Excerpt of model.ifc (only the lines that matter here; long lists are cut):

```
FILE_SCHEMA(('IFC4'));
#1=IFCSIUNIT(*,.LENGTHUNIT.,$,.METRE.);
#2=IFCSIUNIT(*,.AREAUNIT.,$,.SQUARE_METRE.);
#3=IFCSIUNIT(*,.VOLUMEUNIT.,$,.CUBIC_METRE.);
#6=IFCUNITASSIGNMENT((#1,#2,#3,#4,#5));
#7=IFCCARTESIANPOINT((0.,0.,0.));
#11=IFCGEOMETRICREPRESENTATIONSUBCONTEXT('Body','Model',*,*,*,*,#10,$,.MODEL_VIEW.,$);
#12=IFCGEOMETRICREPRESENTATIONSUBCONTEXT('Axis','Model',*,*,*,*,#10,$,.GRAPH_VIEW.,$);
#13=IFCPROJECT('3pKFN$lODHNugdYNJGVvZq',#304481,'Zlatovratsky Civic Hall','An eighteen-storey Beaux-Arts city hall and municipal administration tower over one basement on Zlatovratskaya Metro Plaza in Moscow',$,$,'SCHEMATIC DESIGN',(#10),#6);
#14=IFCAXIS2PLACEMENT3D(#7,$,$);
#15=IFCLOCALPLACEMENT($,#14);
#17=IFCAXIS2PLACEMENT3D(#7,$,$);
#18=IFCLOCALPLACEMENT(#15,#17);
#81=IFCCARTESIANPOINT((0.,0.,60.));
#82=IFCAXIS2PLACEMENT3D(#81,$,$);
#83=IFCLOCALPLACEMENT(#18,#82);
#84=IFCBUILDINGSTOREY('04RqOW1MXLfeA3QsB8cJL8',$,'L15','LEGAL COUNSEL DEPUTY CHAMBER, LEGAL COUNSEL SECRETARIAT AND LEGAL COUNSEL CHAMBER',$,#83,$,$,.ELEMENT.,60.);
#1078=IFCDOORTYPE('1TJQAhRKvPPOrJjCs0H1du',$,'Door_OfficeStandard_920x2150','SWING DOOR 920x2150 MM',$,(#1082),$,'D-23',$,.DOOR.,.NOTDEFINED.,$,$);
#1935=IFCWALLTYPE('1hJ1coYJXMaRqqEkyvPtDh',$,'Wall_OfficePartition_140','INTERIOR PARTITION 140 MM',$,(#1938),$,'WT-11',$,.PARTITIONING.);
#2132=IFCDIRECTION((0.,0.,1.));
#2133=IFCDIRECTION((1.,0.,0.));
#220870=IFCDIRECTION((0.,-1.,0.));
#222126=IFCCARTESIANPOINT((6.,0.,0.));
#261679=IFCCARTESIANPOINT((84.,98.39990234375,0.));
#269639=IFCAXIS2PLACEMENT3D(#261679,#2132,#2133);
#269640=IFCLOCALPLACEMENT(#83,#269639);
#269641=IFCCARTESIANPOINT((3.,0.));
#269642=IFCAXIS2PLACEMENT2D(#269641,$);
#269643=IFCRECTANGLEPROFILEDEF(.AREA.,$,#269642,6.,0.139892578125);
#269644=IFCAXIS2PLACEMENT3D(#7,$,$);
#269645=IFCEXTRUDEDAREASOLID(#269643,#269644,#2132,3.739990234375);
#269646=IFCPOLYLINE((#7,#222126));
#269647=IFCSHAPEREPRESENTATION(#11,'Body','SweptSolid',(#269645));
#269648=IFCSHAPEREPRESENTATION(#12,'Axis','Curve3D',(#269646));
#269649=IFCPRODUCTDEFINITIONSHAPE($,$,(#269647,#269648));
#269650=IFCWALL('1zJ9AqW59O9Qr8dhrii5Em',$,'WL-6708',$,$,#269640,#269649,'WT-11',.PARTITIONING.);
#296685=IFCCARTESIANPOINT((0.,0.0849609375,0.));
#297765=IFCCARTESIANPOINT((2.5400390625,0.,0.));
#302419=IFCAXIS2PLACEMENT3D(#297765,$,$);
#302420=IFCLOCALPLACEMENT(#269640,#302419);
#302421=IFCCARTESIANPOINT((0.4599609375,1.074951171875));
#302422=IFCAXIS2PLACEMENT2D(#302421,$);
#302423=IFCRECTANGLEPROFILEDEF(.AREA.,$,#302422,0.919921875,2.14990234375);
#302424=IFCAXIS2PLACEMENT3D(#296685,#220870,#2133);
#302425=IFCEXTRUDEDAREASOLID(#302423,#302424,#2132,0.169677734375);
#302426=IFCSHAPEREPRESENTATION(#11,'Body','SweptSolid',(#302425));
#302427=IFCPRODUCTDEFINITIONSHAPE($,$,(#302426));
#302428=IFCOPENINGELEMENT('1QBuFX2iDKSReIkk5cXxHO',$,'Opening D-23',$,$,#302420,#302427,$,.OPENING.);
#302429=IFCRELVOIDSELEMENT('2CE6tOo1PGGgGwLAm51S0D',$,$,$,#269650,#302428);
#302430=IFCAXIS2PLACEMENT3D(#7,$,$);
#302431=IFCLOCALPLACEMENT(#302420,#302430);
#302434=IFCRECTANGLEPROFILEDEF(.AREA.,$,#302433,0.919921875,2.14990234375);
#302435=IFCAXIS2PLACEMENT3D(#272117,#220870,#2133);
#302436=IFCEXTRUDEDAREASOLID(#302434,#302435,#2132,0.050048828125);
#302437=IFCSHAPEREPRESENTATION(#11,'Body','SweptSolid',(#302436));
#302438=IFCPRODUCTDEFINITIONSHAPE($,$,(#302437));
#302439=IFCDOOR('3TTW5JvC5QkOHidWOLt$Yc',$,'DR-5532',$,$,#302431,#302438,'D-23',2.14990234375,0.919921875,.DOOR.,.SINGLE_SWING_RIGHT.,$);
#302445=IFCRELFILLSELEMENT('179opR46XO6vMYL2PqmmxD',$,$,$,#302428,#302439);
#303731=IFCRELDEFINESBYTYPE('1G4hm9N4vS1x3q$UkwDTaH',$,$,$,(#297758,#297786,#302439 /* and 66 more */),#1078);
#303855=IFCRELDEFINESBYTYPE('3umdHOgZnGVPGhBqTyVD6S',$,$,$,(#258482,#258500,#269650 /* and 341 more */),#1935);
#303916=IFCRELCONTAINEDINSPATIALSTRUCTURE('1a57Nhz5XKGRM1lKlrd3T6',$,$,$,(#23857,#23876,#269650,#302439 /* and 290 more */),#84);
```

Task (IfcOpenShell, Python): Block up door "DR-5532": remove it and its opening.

```python
import ifcopenshell
import ifcopenshell.api.feature
import ifcopenshell.api.root
import ifcopenshell.geom
import ifcopenshell.util.shape

model = ifcopenshell.open("model.ifc")
settings = ifcopenshell.geom.settings()


def volume(element):
    """Net volume in cubic metres, openings subtracted."""
    shape = ifcopenshell.geom.create_shape(settings, element)
    return ifcopenshell.util.shape.get_volume(shape.geometry)


door = model.by_guid("3TTW5JvC5QkOHidWOLt$Yc")
opening = door.FillsVoids[0].RelatingOpeningElement
wall = opening.VoidsElements[0].RelatingBuildingElement
before = volume(wall)

ifcopenshell.api.root.remove_product(model, product=door)
ifcopenshell.api.feature.remove_feature(model, feature=opening)

after = volume(wall)

print(f"wall volume {before:.3f} -> {after:.3f} m3")

model.write("model-out.ifc")
```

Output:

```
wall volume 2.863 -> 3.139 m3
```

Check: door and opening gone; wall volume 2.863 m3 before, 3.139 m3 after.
